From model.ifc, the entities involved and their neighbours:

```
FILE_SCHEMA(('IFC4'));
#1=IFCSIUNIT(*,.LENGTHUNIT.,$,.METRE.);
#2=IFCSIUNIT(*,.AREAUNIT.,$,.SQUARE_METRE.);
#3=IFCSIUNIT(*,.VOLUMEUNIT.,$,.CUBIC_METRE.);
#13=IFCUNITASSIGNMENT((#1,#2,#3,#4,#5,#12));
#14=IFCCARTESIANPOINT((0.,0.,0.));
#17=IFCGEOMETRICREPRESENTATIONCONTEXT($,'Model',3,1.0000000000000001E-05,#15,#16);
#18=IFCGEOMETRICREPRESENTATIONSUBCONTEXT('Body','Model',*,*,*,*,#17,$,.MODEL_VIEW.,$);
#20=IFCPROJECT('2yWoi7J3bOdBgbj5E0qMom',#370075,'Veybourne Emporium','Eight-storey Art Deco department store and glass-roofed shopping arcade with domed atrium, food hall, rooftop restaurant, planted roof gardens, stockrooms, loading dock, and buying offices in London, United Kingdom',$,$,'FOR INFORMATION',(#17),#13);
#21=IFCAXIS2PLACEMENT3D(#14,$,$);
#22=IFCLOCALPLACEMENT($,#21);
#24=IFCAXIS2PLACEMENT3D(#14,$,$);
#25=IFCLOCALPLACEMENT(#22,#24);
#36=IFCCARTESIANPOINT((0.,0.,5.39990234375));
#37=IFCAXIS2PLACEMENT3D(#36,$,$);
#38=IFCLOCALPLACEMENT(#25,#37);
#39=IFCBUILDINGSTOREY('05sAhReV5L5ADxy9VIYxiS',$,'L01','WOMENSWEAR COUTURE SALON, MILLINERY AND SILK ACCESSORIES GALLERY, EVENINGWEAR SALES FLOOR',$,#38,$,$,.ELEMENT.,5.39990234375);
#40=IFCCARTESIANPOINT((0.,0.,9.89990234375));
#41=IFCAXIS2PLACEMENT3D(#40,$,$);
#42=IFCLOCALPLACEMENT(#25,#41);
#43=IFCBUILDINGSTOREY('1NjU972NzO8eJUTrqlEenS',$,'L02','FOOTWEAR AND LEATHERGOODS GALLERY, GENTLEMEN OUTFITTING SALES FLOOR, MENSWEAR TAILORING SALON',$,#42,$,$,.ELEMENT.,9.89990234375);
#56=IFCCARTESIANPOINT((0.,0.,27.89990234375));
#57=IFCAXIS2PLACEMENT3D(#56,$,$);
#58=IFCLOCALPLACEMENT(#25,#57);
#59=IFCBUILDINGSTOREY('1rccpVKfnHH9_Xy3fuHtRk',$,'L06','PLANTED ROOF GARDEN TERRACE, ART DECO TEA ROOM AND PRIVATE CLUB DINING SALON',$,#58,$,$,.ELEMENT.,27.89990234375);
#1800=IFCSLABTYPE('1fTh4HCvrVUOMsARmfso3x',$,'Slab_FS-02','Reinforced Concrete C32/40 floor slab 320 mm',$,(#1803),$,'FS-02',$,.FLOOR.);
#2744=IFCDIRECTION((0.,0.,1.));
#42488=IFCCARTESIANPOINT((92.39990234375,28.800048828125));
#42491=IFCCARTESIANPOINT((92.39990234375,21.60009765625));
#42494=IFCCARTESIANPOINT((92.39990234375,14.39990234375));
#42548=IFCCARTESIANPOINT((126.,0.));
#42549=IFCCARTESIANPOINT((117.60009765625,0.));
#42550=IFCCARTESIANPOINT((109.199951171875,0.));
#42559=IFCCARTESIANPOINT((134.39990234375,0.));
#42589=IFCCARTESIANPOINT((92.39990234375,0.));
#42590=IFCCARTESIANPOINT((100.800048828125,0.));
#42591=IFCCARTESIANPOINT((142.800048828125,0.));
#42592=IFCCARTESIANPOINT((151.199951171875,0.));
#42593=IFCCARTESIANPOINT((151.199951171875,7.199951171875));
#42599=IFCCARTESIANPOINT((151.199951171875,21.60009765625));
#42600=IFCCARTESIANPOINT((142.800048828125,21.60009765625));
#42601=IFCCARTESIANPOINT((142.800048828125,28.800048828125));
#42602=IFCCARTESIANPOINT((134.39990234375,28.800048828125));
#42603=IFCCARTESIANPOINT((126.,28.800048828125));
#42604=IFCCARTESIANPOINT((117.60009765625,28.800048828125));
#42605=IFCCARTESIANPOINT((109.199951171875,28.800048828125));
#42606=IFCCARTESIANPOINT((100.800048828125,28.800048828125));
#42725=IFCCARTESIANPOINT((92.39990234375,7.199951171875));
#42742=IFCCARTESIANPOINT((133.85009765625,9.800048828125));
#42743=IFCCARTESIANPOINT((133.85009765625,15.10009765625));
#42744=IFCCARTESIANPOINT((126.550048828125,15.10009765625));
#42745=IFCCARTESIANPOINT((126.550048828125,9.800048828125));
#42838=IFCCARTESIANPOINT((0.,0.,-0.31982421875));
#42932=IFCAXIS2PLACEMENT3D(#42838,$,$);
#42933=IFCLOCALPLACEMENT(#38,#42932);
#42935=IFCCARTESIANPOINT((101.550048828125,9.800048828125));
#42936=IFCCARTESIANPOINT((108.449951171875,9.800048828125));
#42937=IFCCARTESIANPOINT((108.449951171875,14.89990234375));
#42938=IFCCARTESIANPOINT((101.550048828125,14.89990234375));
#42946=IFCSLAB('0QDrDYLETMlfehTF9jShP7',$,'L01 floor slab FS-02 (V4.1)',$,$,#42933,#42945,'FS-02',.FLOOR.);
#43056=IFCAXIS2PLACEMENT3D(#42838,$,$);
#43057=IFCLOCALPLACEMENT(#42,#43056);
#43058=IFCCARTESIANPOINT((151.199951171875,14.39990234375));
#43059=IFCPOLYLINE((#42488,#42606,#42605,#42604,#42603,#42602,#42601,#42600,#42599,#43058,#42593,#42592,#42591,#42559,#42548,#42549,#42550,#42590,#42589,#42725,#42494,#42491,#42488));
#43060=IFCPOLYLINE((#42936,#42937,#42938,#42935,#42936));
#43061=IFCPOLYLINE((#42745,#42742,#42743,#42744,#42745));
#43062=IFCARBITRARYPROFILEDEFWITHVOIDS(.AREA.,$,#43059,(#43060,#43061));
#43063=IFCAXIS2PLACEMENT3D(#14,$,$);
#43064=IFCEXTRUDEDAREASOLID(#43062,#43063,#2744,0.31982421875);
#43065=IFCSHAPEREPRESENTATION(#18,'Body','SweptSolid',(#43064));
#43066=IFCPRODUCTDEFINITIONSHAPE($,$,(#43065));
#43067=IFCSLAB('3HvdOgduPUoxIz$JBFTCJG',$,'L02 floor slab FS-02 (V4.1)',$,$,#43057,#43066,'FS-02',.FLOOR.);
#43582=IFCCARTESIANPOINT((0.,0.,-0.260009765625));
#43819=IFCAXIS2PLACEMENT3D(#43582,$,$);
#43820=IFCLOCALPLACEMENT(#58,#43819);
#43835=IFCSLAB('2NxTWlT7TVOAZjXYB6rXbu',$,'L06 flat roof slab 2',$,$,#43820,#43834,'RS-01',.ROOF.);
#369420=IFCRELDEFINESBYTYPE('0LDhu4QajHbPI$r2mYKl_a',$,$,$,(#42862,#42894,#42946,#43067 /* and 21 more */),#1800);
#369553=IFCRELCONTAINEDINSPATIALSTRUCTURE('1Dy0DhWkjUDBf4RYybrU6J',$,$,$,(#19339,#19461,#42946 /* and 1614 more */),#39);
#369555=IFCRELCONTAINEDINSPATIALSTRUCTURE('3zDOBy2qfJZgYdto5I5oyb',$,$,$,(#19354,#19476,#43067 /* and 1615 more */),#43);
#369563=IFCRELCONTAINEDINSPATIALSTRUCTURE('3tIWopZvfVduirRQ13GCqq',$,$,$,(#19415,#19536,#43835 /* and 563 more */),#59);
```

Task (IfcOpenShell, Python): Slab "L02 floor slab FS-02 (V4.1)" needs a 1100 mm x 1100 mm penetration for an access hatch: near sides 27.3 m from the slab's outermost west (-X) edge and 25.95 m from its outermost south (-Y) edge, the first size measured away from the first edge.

```python
import numpy as np
import ifcopenshell
import ifcopenshell.api.feature
import ifcopenshell.api.geometry
import ifcopenshell.api.root
import ifcopenshell.geom
import ifcopenshell.util.placement
import ifcopenshell.util.representation
import ifcopenshell.util.shape
import ifcopenshell.util.unit

model = ifcopenshell.open("model.ifc")
unit_scale = ifcopenshell.util.unit.calculate_unit_scale(model)
settings = ifcopenshell.geom.settings()


def volume(element):
    """Net volume in cubic metres, openings subtracted."""
    shape = ifcopenshell.geom.create_shape(settings, element)
    return ifcopenshell.util.shape.get_volume(shape.geometry)


slab = model.by_guid("3HvdOgduPUoxIz$JBFTCJG")
before = volume(slab)

# Extent in the slab's own axes, in metres. The edges named are its -X and -Y sides.
slab_shape = ifcopenshell.geom.create_shape(settings, slab)
vertices = ifcopenshell.util.shape.get_vertices(slab_shape.geometry)
x_min, y_min, bottom = vertices.min(axis=0)
top = vertices[:, 2].max()

opening = ifcopenshell.api.root.create_entity(model, ifc_class="IfcOpeningElement", name="Access hatch opening", predefined_type="OPENING")
context = ifcopenshell.util.representation.get_context(model, "Model", "Body", "MODEL_VIEW")
width, depth = 1.1, 1.1
outline = [(0.0, 0.0), (width, 0.0), (width, depth), (0.0, depth), (0.0, 0.0)]
# Overshoot both faces by 50 mm so the cut is clean.
shape = ifcopenshell.api.geometry.add_slab_representation(
    model, context=context, depth=top - bottom + 0.1, polyline=outline
)
ifcopenshell.api.geometry.assign_representation(model, product=opening, representation=shape)

matrix = ifcopenshell.util.placement.get_local_placement(slab.ObjectPlacement)
matrix[:, 3] = matrix @ np.append(np.array([x_min + 27.3, y_min + 25.95, bottom - 0.05]) / unit_scale, 1.0)
ifcopenshell.api.geometry.edit_object_placement(model, product=opening, matrix=matrix, is_si=False)
ifcopenshell.api.feature.add_feature(model, feature=opening, element=slab)

after = volume(slab)

print(f"slab volume {before:.3f} -> {after:.3f} m3")

model.write("model_edited.ifc")
```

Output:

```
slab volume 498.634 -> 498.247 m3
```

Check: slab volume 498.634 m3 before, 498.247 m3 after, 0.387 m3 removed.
